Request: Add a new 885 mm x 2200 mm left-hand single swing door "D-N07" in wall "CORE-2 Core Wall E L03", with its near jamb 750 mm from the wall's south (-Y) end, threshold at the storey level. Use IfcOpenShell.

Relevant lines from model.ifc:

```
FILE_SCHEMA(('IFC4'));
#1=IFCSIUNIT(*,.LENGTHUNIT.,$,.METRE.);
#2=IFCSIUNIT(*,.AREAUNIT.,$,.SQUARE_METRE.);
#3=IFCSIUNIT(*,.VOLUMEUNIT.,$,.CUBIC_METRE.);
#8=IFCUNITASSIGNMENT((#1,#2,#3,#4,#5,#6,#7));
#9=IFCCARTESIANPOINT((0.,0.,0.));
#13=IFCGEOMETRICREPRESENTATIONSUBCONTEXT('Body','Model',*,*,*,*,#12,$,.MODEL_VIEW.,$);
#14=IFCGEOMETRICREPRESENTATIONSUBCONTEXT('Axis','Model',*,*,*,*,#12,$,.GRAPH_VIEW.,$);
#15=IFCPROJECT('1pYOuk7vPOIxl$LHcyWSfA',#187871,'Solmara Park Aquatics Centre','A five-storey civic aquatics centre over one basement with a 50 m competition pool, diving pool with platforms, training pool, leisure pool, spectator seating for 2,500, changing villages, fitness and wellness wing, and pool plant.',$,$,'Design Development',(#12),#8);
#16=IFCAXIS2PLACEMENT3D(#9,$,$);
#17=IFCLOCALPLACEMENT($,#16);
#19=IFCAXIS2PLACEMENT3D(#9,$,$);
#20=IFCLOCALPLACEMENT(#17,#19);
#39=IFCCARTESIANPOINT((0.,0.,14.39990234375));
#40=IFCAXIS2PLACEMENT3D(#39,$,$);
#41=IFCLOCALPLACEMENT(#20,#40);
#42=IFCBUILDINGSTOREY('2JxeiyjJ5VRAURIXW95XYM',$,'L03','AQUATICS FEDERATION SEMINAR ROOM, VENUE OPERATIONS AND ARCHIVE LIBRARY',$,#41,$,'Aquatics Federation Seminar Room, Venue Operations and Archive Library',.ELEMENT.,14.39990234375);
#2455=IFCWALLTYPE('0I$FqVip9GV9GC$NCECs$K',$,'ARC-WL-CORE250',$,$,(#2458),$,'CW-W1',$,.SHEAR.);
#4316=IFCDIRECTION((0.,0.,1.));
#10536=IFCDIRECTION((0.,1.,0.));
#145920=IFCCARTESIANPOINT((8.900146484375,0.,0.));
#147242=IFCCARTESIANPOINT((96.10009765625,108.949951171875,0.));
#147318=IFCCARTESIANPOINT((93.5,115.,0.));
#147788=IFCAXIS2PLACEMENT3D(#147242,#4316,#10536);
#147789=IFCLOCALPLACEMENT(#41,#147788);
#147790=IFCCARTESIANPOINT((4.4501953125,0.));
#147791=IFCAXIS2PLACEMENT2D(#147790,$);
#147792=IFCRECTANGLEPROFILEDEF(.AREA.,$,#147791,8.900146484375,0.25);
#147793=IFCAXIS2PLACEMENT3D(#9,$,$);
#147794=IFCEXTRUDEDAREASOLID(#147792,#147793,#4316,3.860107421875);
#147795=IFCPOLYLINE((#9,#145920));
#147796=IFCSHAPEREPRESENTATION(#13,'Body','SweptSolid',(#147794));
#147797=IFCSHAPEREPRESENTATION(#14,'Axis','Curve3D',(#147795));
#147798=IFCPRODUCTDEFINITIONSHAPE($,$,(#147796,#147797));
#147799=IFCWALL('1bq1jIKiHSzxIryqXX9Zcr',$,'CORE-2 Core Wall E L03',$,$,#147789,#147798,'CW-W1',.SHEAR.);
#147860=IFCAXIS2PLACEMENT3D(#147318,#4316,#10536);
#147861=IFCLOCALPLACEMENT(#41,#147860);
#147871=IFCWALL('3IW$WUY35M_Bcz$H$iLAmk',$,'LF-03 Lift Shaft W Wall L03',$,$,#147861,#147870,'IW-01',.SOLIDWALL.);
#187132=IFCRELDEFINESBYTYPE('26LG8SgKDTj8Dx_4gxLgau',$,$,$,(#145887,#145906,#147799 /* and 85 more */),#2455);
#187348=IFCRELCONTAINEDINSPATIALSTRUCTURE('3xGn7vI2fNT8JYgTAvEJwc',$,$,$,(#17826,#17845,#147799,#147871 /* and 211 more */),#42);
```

```python
import numpy as np
import ifcopenshell
import ifcopenshell.api.feature
import ifcopenshell.api.geometry
import ifcopenshell.api.root
import ifcopenshell.api.spatial
import ifcopenshell.geom
import ifcopenshell.util.element
import ifcopenshell.util.placement
import ifcopenshell.util.representation
import ifcopenshell.util.shape
import ifcopenshell.util.unit

model = ifcopenshell.open("model.ifc")
unit_scale = ifcopenshell.util.unit.calculate_unit_scale(model)
settings = ifcopenshell.geom.settings()


def volume(element):
    """Net volume in cubic metres, openings subtracted."""
    shape = ifcopenshell.geom.create_shape(settings, element)
    return ifcopenshell.util.shape.get_volume(shape.geometry)


wall = model.by_guid("1bq1jIKiHSzxIryqXX9Zcr")
storey = ifcopenshell.util.element.get_container(wall, ifc_class="IfcBuildingStorey")
context = ifcopenshell.util.representation.get_context(model, "Model", "Body", "MODEL_VIEW")
before = volume(wall)

width, height, from_end, sill = 0.885, 2.2, 0.75, 0.0  # metres

# The wall runs along its own X axis, and the end named is its -X end.
wall_shape = ifcopenshell.geom.create_shape(settings, wall)
x, y, z = ifcopenshell.util.shape.get_vertices(wall_shape.geometry).T
start = x.min() + from_end
face, thickness = float(y.min()), float(y.max() - y.min())
wall_matrix = ifcopenshell.util.placement.get_local_placement(wall.ObjectPlacement)
level = ifcopenshell.util.placement.get_local_placement(storey.ObjectPlacement)[2, 3]


def in_wall(x, y):
    """Placement at x, y metres in the wall's axes, at sill height."""
    matrix = wall_matrix.copy()
    matrix[:, 3] = wall_matrix @ np.array([x / unit_scale, y / unit_scale, 0.0, 1.0])
    matrix[2, 3] = level + sill / unit_scale
    return matrix


# Opening: a box that overshoots both wall faces by 50 mm.
opening = ifcopenshell.api.root.create_entity(model, ifc_class="IfcOpeningElement", predefined_type="OPENING")
box = ifcopenshell.api.geometry.add_wall_representation(
    model, context=context, length=width, height=height, thickness=thickness + 0.1
)
ifcopenshell.api.geometry.assign_representation(model, product=opening, representation=box)
ifcopenshell.api.geometry.edit_object_placement(model, product=opening, matrix=in_wall(start, face - 0.05), is_si=False)
ifcopenshell.api.feature.add_feature(model, feature=opening, element=wall)

door = ifcopenshell.api.root.create_entity(model, ifc_class="IfcDoor", name="D-N07", predefined_type="DOOR")
door.OverallWidth, door.OverallHeight = width / unit_scale, height / unit_scale
door.OperationType = "SINGLE_SWING_LEFT"
body = ifcopenshell.api.geometry.add_door_representation(
    model,
    context=context,
    overall_width=door.OverallWidth,
    overall_height=door.OverallHeight,
    operation_type="SINGLE_SWING_LEFT",
    lining_properties={"LiningDepth": thickness / unit_scale, "ThresholdDepth": thickness / unit_scale},
)
ifcopenshell.api.geometry.assign_representation(model, product=door, representation=body)
ifcopenshell.api.spatial.assign_container(model, products=[door], relating_structure=storey)
ifcopenshell.api.feature.add_filling(model, opening=opening, element=door)

# The lining spans the wall, so the door starts at the wall face.
ifcopenshell.api.geometry.edit_object_placement(model, product=door, matrix=in_wall(start, face), is_si=False)

after = volume(wall)

print(f"wall volume {before:.3f} -> {after:.3f} m3")

model.write("model_updated.ifc")
```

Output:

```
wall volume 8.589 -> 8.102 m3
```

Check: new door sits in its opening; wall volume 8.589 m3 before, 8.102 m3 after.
